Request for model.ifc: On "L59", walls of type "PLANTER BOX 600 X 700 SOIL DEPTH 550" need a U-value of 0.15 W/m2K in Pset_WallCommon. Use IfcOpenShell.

First a look at what the model holds.

```python
import ifcopenshell
import ifcopenshell.util.element

model = ifcopenshell.open("model.ifc")
print(model.schema)
storey = next(s for s in model.by_type("IfcBuildingStorey") if s.Name == "L59")
walls = [e for e in ifcopenshell.util.element.get_decomposition(storey) if e.is_a("IfcWall")]
seen = {}
for e in walls:
    element_type = ifcopenshell.util.element.get_type(e)
    key = (element_type.Name if element_type != e and element_type else None, ifcopenshell.util.element.get_pset(e, "Pset_WallCommon", "ThermalTransmittance"))
    seen[key] = seen.get(key, 0) + 1
for (name, value), count in sorted(seen.items(), key=str):
    print(count, "x", name, "|", value)
```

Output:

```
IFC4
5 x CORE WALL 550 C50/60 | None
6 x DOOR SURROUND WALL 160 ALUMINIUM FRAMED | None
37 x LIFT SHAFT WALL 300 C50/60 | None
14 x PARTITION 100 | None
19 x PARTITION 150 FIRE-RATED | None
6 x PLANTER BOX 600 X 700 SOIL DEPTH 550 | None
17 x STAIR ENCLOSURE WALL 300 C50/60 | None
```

```python
import ifcopenshell
import ifcopenshell.api.pset
import ifcopenshell.util.element

model = ifcopenshell.open("model.ifc")

storey = next(s for s in model.by_type("IfcBuildingStorey") if s.Name == "L59")
walls = [e for e in ifcopenshell.util.element.get_decomposition(storey) if e.is_a("IfcWall")]

count = 0
for e in walls:
    element_type = ifcopenshell.util.element.get_type(e)
    if element_type in (None, e) or element_type.Name != "PLANTER BOX 600 X 700 SOIL DEPTH 550":
        continue
    found = ifcopenshell.util.element.get_pset(e, "Pset_WallCommon", should_inherit=False)
    if found:
        pset = model.by_id(found["id"])
        if len(ifcopenshell.util.element.get_elements_by_pset(pset)) > 1:
            pset = ifcopenshell.api.pset.unshare_pset(model, products=[e], pset=pset)[0]
    else:
        pset = ifcopenshell.api.pset.add_pset(model, product=e, name="Pset_WallCommon")
    ifcopenshell.api.pset.edit_pset(model, pset=pset, properties={"ThermalTransmittance": 0.15})
    count += 1

print(count, "walls updated")

model.write("model_rev.ifc")
```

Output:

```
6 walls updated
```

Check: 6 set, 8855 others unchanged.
